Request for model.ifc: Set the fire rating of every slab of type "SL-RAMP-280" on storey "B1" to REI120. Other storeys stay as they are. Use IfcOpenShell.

First a look at what the model holds.

```python
import ifcopenshell
import ifcopenshell.util.element

model = ifcopenshell.open("model.ifc")
print(model.schema)
storey = next(s for s in model.by_type("IfcBuildingStorey") if s.Name == "B1")
slabs = [e for e in ifcopenshell.util.element.get_decomposition(storey) if e.is_a("IfcSlab")]
seen = {}
for e in slabs:
    element_type = ifcopenshell.util.element.get_type(e)
    key = (element_type.Name if element_type != e and element_type else None, ifcopenshell.util.element.get_pset(e, "Pset_SlabCommon", "FireRating"))
    seen[key] = seen.get(key, 0) + 1
for (name, value), count in sorted(seen.items(), key=str):
    print(count, "x", name, "|", value)
```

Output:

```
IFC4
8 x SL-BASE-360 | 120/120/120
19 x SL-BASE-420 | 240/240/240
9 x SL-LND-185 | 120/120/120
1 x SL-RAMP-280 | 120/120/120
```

```python
import ifcopenshell
import ifcopenshell.api.pset
import ifcopenshell.util.element

model = ifcopenshell.open("model.ifc")

storey = next(s for s in model.by_type("IfcBuildingStorey") if s.Name == "B1")
slabs = [e for e in ifcopenshell.util.element.get_decomposition(storey) if e.is_a("IfcSlab")]

count = 0
for e in slabs:
    element_type = ifcopenshell.util.element.get_type(e)
    if element_type in (None, e) or element_type.Name != "SL-RAMP-280":
        continue
    # add_pset returns the element's existing set when there is one.
    pset = ifcopenshell.api.pset.add_pset(model, product=e, name="Pset_SlabCommon")
    ifcopenshell.api.pset.edit_pset(model, pset=pset, properties={"FireRating": "REI120"})
    count += 1

print(count, "slabs updated")

model.write("model_updated.ifc")
```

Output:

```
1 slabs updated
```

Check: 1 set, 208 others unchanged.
